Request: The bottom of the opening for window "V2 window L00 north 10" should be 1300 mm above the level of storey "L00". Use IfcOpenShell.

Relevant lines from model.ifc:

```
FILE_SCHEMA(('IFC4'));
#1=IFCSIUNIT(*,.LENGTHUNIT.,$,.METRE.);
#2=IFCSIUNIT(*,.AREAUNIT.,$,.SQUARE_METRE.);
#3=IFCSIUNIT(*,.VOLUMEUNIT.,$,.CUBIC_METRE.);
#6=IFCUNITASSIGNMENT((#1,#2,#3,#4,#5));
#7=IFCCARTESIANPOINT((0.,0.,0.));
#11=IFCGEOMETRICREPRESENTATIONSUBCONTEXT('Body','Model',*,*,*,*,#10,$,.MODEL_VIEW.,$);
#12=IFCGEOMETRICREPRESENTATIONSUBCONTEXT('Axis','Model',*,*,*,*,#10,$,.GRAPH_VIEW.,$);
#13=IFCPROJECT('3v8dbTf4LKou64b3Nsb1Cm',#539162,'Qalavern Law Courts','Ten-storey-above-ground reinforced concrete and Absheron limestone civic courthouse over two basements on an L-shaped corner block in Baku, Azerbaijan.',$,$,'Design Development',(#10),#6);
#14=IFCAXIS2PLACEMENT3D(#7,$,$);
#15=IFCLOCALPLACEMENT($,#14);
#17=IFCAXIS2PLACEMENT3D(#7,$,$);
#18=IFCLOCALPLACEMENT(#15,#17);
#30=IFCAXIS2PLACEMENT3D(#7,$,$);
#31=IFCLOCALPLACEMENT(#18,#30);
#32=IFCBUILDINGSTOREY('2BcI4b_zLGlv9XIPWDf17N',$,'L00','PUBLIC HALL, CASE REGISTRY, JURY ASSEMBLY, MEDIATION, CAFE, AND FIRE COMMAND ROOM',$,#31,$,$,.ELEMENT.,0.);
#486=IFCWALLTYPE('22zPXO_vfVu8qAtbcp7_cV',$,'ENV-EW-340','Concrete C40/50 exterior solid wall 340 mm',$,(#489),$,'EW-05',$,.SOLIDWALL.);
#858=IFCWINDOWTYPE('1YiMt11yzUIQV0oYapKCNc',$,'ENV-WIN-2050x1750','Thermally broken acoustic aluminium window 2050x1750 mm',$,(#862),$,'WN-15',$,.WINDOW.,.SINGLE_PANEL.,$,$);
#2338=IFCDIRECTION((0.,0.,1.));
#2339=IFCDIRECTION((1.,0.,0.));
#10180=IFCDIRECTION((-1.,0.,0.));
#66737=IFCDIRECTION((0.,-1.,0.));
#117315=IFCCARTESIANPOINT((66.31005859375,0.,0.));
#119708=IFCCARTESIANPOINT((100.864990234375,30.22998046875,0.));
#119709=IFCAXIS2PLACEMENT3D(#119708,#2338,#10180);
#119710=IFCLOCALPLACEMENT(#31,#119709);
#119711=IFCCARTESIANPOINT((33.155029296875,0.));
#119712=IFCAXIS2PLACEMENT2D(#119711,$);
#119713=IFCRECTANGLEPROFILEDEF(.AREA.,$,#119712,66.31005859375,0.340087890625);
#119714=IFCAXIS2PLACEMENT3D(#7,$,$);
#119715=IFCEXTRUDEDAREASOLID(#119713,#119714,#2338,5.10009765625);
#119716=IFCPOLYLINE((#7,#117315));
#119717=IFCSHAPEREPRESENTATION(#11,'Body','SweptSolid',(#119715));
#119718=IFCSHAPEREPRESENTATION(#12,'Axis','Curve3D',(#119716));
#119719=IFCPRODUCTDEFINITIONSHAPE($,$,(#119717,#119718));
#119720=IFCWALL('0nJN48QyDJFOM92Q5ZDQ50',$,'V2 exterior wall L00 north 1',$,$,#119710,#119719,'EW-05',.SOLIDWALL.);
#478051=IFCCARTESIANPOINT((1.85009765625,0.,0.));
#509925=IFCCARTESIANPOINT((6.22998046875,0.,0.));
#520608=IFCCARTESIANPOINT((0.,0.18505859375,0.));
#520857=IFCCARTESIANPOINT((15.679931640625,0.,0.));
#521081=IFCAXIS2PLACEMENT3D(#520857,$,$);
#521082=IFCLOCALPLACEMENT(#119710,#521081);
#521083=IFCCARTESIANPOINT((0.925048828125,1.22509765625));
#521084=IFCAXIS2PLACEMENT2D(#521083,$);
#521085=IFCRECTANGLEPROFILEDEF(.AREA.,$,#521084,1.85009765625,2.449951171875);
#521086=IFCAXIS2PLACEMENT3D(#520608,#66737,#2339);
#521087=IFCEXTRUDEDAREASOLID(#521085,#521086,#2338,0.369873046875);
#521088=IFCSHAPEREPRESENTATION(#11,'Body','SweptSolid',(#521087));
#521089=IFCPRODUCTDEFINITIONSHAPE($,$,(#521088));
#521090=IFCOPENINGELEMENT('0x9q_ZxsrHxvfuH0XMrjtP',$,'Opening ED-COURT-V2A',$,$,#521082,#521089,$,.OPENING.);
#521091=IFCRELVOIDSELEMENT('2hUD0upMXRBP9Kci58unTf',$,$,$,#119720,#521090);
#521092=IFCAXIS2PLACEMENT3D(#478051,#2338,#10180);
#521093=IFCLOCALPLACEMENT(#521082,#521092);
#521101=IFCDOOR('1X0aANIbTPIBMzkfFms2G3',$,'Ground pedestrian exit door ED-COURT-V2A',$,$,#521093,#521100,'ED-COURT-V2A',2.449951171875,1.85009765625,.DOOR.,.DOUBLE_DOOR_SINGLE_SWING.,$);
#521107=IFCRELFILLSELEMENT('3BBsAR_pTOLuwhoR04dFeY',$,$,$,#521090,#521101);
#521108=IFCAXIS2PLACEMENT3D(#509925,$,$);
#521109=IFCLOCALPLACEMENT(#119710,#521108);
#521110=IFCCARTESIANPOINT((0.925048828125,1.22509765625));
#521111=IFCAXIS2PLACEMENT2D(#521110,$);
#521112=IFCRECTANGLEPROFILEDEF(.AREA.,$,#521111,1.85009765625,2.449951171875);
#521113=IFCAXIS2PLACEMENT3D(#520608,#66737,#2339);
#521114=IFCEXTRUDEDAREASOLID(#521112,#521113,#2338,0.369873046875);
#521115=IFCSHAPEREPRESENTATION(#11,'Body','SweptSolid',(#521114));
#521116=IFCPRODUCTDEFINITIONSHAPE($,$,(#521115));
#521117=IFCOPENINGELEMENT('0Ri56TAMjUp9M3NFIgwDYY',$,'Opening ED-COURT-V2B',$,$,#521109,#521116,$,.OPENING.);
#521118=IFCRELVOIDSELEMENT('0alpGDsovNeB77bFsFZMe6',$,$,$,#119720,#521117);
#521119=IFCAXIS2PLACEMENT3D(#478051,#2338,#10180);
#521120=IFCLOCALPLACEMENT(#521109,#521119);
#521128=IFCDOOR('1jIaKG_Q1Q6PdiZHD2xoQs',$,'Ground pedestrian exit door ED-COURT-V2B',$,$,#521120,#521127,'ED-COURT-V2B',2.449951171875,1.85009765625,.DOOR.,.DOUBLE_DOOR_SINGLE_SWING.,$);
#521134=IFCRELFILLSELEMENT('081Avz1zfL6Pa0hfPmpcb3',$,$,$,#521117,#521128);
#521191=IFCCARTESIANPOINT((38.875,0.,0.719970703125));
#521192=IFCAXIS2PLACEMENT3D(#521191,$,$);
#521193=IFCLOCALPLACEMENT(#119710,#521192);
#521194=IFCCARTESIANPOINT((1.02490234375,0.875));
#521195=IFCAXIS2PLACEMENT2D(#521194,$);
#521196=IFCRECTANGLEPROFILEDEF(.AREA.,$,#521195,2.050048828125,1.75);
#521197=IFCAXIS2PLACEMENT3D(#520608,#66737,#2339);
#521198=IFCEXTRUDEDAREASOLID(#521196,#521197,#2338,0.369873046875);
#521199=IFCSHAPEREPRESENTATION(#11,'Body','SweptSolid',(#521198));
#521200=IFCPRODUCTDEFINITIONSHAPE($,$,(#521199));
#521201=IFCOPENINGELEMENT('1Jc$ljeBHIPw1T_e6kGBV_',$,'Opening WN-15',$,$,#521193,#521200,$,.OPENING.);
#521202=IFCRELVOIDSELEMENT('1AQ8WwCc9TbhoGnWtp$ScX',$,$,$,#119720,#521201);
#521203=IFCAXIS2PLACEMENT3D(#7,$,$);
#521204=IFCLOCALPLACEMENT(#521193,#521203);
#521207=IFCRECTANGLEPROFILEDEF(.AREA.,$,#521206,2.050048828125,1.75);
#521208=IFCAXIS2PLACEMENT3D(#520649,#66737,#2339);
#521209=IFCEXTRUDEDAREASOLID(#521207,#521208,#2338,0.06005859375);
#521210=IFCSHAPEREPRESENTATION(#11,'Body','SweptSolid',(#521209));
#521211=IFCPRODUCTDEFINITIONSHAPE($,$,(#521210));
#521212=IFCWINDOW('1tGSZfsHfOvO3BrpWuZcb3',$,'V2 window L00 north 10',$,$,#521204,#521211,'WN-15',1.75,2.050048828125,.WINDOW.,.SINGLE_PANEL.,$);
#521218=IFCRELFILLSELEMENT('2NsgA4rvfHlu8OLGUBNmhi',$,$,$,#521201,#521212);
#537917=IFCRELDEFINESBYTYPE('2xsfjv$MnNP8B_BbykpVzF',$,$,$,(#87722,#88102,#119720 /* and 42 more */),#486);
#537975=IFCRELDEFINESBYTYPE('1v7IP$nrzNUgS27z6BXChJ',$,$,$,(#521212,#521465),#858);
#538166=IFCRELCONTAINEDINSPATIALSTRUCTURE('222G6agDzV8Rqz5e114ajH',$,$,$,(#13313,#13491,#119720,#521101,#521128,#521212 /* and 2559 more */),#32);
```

```python
import numpy as np
import ifcopenshell
import ifcopenshell.api.geometry
import ifcopenshell.geom
import ifcopenshell.util.element
import ifcopenshell.util.placement
import ifcopenshell.util.shape
import ifcopenshell.util.unit

model = ifcopenshell.open("model.ifc")
unit_scale = ifcopenshell.util.unit.calculate_unit_scale(model)

window = model.by_guid("1tGSZfsHfOvO3BrpWuZcb3")
opening = window.FillsVoids[0].RelatingOpeningElement
storey = ifcopenshell.util.element.get_container(window, ifc_class="IfcBuildingStorey")
level = ifcopenshell.util.placement.get_local_placement(storey.ObjectPlacement)[2, 3]

# The opening's origin need not be at the sill, so measure its lowest point.
shape = ifcopenshell.geom.create_shape(ifcopenshell.geom.settings(), opening)
bottom = ifcopenshell.util.shape.get_shape_bottom_elevation(shape, shape.geometry) / unit_scale
dz = level + 1.3 / unit_scale - bottom

shift = np.array([0.0, 0.0, dz])
# The window is placed relative to its opening, so it follows when the opening moves.
matrix = ifcopenshell.util.placement.get_local_placement(opening.ObjectPlacement)
matrix[:3, 3] += shift
ifcopenshell.api.geometry.edit_object_placement(
    model, product=opening, matrix=matrix, is_si=False, should_transform_children=True
)

print(f"moved by {dz * unit_scale:+.3f} m")

model.write("model_updated.ifc")
```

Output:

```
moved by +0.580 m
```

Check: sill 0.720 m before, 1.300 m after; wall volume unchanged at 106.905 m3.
